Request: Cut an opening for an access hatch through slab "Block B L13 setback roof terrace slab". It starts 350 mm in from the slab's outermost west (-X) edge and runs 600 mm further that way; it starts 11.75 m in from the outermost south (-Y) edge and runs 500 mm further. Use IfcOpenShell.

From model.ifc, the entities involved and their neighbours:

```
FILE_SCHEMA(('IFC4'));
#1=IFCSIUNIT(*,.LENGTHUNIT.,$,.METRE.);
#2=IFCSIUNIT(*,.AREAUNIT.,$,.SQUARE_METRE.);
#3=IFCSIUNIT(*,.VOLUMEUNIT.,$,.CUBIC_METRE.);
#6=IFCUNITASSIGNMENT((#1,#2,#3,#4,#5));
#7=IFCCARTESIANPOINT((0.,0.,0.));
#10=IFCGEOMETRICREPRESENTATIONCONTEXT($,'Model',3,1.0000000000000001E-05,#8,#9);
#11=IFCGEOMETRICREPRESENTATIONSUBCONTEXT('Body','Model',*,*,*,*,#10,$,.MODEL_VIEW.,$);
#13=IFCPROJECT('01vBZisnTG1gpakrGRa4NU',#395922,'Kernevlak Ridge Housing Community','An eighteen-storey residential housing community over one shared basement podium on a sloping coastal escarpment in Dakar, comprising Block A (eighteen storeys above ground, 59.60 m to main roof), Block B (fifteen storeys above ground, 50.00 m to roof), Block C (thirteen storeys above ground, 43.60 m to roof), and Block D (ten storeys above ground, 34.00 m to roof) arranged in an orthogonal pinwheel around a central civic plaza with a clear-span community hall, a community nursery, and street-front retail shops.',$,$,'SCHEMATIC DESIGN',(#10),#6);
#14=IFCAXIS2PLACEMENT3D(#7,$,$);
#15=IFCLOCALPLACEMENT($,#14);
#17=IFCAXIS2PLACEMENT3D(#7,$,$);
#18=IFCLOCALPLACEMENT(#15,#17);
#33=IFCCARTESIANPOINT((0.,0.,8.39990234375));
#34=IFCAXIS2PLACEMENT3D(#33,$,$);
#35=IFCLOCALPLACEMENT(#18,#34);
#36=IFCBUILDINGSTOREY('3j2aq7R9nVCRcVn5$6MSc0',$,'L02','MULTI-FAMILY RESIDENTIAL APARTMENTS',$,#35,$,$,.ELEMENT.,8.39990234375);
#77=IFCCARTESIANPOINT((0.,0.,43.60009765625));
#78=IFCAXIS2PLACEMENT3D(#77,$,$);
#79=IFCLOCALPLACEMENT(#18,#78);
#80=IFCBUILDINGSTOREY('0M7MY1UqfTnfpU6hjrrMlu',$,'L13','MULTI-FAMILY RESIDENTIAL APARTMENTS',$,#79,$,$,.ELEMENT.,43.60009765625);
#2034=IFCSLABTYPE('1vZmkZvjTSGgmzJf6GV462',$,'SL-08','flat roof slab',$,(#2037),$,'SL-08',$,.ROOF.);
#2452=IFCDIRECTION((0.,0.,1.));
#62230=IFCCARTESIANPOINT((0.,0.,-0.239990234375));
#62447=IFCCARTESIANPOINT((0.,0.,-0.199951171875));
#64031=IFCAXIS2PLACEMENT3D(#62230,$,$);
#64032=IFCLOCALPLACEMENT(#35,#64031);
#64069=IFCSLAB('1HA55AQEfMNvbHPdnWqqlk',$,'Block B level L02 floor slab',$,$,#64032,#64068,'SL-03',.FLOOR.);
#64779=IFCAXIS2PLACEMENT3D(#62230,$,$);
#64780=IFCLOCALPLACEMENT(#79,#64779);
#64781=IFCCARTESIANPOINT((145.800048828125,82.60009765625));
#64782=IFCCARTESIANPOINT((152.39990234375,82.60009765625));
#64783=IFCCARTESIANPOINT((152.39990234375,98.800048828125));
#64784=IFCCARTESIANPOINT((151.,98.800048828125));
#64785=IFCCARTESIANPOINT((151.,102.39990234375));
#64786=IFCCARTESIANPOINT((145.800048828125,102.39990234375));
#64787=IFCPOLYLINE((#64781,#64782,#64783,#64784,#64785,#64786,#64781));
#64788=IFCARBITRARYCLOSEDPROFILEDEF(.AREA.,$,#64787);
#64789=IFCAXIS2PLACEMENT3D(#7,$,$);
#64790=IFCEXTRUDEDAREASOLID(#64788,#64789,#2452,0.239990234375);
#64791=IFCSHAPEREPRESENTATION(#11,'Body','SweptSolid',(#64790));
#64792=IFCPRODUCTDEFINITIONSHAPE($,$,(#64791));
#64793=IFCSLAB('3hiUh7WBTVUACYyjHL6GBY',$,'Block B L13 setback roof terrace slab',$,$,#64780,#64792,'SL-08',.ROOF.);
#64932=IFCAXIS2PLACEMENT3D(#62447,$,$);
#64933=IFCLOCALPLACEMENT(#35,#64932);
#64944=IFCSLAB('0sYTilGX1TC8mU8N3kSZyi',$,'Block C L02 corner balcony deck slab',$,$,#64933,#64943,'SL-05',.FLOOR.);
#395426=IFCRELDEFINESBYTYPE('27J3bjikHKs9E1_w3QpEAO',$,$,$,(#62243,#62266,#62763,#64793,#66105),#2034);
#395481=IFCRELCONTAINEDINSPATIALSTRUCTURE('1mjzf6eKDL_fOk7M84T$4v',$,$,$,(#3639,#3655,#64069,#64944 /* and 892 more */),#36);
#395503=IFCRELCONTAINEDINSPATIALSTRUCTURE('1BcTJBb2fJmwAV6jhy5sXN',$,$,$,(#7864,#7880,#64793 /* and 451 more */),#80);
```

```python
import numpy as np
import ifcopenshell
import ifcopenshell.api.feature
import ifcopenshell.api.geometry
import ifcopenshell.api.root
import ifcopenshell.geom
import ifcopenshell.util.placement
import ifcopenshell.util.representation
import ifcopenshell.util.shape
import ifcopenshell.util.unit

model = ifcopenshell.open("model.ifc")
unit_scale = ifcopenshell.util.unit.calculate_unit_scale(model)
settings = ifcopenshell.geom.settings()


def volume(element):
    """Net volume in cubic metres, openings subtracted."""
    shape = ifcopenshell.geom.create_shape(settings, element)
    return ifcopenshell.util.shape.get_volume(shape.geometry)


slab = model.by_id(64793)
before = volume(slab)

# Extent in the slab's own axes, in metres. The edges named are its -X and -Y sides.
slab_shape = ifcopenshell.geom.create_shape(settings, slab)
vertices = ifcopenshell.util.shape.get_vertices(slab_shape.geometry)
x_min, y_min, bottom = vertices.min(axis=0)
top = vertices[:, 2].max()

opening = ifcopenshell.api.root.create_entity(model, ifc_class="IfcOpeningElement", name="Access hatch opening", predefined_type="OPENING")
context = ifcopenshell.util.representation.get_context(model, "Model", "Body", "MODEL_VIEW")
width, depth = 0.6, 0.5
outline = [(0.0, 0.0), (width, 0.0), (width, depth), (0.0, depth), (0.0, 0.0)]
# Overshoot both faces by 50 mm so the cut is clean.
shape = ifcopenshell.api.geometry.add_slab_representation(
    model, context=context, depth=top - bottom + 0.1, polyline=outline
)
ifcopenshell.api.geometry.assign_representation(model, product=opening, representation=shape)

matrix = ifcopenshell.util.placement.get_local_placement(slab.ObjectPlacement)
matrix[:, 3] = matrix @ np.append(np.array([x_min + 0.35, y_min + 11.75, bottom - 0.05]) / unit_scale, 1.0)
ifcopenshell.api.geometry.edit_object_placement(model, product=opening, matrix=matrix, is_si=False)
ifcopenshell.api.feature.add_feature(model, feature=opening, element=slab)

after = volume(slab)

print(f"slab volume {before:.3f} -> {after:.3f} m3")

model.write("model_v2.ifc")
```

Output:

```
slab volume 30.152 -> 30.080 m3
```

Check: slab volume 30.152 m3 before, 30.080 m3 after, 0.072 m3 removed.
